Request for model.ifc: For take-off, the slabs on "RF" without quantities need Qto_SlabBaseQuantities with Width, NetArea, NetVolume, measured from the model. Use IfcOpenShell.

First a look at what the model holds.

```python
import ifcopenshell
import ifcopenshell.util.element
import ifcopenshell.util.unit

model = ifcopenshell.open("model.ifc")
print(model.schema)
for unit_type in ("LENGTHUNIT", "AREAUNIT", "VOLUMEUNIT"):
    print(unit_type, ifcopenshell.util.unit.calculate_unit_scale(model, unit_type))
storey = next(s for s in model.by_type("IfcBuildingStorey") if s.Name == "RF")
slabs = [e for e in ifcopenshell.util.element.get_decomposition(storey) if e.is_a("IfcSlab")]
for e in sorted(slabs, key=lambda e: e.id()):
    print(e.id(), e.is_a(), e.Name, list(ifcopenshell.util.element.get_psets(e, qtos_only=True)), sep=" | ")
```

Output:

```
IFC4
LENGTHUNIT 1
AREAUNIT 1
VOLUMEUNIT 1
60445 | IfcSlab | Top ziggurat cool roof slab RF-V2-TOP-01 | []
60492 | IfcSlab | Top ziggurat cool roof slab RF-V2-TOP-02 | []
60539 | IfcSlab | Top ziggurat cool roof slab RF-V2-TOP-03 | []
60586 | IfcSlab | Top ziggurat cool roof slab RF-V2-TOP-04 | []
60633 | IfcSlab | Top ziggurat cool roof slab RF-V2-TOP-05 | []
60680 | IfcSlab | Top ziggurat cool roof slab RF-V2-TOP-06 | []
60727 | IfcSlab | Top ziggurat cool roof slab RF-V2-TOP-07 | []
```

```python
import ifcopenshell
import ifcopenshell.api.pset
import ifcopenshell.geom
import ifcopenshell.util.element
import ifcopenshell.util.shape
import ifcopenshell.util.unit

model = ifcopenshell.open("model.ifc")
unit_scale = ifcopenshell.util.unit.calculate_unit_scale(model)
area_scale = ifcopenshell.util.unit.calculate_unit_scale(model, "AREAUNIT")
volume_scale = ifcopenshell.util.unit.calculate_unit_scale(model, "VOLUMEUNIT")
settings = ifcopenshell.geom.settings()

storey = next(s for s in model.by_type("IfcBuildingStorey") if s.Name == "RF")
slabs = [e for e in ifcopenshell.util.element.get_decomposition(storey) if e.is_a("IfcSlab")]

for e in sorted(slabs, key=lambda e: e.id()):
    if ifcopenshell.util.element.get_psets(e, qtos_only=True, should_inherit=False):
        continue
    # Geometry comes back in metres, in the element's own axes.
    shape = ifcopenshell.geom.create_shape(settings, e)
    values = {
        "Width": ifcopenshell.util.shape.get_z(shape.geometry) / unit_scale,
        "NetArea": ifcopenshell.util.shape.get_footprint_area(shape.geometry) / area_scale,
        "NetVolume": ifcopenshell.util.shape.get_volume(shape.geometry) / volume_scale,
    }
    qto = ifcopenshell.api.pset.add_qto(model, product=e, name="Qto_SlabBaseQuantities")
    ifcopenshell.api.pset.edit_qto(model, qto=qto, properties=values)
    print(e.id(), {k: round(v, 3) for k, v in values.items()})

model.write("model_v2.ifc")
```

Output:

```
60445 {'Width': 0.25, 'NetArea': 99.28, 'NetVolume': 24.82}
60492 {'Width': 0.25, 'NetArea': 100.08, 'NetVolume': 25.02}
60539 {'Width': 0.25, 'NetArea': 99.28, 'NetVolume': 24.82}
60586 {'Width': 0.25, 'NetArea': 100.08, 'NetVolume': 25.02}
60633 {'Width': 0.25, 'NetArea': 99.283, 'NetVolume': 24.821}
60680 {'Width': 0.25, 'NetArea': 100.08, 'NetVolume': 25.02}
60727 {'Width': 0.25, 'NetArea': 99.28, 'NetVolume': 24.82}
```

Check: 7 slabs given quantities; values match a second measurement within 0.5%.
